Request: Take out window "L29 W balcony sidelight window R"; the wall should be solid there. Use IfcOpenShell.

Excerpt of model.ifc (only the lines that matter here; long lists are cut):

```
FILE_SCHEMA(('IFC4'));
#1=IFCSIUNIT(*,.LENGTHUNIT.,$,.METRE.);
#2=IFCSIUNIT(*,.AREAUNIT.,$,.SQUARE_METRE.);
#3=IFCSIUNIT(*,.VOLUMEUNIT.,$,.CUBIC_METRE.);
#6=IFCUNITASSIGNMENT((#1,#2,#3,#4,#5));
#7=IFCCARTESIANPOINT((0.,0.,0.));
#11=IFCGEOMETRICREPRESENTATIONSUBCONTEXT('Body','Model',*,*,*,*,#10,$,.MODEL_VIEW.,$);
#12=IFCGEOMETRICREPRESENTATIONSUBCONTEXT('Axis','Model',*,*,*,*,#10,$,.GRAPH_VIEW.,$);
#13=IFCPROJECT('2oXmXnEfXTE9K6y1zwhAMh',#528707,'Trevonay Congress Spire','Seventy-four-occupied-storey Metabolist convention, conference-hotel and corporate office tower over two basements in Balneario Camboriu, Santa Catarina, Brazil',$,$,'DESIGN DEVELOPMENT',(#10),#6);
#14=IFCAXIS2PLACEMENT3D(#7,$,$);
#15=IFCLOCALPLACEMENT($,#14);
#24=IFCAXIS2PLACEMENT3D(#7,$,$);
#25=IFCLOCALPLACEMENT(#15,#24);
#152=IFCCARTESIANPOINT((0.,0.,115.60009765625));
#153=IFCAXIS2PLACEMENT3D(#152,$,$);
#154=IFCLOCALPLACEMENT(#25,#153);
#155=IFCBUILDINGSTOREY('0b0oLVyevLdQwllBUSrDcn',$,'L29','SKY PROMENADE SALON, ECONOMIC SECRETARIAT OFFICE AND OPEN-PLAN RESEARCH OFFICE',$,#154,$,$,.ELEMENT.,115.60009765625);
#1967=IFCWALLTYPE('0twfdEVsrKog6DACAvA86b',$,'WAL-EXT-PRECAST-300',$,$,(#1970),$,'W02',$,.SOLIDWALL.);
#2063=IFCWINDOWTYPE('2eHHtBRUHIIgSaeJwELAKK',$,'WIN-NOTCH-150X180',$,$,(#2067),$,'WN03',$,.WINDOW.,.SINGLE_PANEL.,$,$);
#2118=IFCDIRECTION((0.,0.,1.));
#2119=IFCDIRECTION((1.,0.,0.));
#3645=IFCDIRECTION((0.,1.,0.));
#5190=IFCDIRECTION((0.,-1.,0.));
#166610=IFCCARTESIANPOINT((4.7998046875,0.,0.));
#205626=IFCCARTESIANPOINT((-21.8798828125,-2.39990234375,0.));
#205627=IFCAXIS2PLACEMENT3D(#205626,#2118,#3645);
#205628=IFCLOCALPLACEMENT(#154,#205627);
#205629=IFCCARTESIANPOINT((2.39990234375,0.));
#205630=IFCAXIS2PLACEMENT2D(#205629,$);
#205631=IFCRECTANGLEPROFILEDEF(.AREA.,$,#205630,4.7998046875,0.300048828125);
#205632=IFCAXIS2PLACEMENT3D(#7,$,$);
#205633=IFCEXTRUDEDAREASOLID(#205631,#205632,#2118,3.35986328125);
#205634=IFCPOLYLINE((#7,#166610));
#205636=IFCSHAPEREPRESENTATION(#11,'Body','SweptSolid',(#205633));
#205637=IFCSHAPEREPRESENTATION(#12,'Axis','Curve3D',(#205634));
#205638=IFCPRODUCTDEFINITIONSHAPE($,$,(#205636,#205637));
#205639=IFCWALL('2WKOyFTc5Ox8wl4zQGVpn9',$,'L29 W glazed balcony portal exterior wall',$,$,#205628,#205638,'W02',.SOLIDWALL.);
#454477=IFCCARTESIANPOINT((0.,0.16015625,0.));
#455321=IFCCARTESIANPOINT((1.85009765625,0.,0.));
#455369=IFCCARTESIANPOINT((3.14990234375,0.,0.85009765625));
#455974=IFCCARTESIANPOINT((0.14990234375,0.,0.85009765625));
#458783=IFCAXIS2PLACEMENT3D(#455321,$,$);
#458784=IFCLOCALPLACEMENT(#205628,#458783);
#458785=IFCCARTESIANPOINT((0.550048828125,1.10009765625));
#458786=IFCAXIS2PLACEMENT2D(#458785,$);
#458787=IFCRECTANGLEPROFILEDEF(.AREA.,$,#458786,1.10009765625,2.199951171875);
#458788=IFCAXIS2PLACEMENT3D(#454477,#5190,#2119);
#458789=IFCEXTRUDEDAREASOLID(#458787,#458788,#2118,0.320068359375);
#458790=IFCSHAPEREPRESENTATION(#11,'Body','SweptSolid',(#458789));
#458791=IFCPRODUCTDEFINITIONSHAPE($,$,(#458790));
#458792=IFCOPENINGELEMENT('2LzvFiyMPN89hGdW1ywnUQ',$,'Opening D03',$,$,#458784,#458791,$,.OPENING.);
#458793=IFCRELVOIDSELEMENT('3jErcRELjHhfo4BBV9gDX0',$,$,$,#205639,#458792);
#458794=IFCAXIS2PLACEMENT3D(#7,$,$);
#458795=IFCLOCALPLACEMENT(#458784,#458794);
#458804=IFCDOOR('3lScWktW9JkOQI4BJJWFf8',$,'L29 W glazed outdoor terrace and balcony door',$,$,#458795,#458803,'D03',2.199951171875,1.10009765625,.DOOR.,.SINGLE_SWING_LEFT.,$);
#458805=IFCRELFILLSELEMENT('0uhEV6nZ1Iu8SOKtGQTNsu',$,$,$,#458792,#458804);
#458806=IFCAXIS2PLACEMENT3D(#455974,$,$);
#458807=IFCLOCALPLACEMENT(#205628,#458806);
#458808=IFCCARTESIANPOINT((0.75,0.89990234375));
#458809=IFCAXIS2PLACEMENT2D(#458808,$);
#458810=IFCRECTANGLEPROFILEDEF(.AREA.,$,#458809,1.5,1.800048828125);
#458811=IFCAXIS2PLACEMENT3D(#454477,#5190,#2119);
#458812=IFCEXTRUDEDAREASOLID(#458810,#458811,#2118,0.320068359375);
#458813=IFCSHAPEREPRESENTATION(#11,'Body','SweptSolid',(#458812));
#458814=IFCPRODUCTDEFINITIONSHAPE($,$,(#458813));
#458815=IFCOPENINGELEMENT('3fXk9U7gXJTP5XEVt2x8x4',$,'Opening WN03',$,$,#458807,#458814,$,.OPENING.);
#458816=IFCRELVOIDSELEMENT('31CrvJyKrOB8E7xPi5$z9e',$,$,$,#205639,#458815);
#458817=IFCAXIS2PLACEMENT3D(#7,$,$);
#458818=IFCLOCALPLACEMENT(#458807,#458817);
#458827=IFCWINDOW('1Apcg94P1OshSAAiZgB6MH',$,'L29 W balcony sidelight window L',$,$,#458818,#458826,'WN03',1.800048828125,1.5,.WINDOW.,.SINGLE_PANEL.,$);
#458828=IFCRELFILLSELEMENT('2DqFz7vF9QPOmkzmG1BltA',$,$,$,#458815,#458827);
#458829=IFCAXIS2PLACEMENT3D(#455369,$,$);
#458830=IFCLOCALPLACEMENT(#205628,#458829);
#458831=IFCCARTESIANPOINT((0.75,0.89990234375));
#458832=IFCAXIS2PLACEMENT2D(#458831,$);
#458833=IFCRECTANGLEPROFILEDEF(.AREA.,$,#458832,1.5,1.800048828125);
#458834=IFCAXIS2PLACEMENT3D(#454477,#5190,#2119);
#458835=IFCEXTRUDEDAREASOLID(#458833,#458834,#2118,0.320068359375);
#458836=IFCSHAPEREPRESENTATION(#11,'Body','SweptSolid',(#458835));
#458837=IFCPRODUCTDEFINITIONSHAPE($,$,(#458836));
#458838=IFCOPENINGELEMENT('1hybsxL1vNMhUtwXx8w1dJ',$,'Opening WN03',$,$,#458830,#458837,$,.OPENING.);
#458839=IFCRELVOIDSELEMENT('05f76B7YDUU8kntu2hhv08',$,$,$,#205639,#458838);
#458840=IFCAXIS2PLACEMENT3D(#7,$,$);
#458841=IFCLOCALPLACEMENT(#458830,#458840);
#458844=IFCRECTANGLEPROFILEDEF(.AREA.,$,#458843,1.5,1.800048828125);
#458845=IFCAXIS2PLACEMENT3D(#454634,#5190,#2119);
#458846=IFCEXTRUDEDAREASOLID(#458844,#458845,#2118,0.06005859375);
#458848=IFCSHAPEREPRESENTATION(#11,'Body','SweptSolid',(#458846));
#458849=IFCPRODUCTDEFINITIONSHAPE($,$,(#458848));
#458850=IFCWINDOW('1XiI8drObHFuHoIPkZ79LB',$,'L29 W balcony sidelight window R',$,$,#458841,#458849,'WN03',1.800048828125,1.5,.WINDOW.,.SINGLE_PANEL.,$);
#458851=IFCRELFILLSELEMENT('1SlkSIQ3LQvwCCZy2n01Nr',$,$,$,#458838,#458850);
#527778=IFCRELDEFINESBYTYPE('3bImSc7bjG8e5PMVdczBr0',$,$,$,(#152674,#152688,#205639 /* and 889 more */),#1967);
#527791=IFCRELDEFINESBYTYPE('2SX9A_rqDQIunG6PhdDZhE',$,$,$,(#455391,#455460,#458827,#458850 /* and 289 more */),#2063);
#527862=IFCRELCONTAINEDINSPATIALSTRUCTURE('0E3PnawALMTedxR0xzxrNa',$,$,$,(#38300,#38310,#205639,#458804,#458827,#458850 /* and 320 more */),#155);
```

```python
import ifcopenshell
import ifcopenshell.api.feature
import ifcopenshell.api.root
import ifcopenshell.geom
import ifcopenshell.util.shape

model = ifcopenshell.open("model.ifc")
settings = ifcopenshell.geom.settings()


def volume(element):
    """Net volume in cubic metres, openings subtracted."""
    shape = ifcopenshell.geom.create_shape(settings, element)
    return ifcopenshell.util.shape.get_volume(shape.geometry)


window = model.by_guid("1XiI8drObHFuHoIPkZ79LB")
opening = window.FillsVoids[0].RelatingOpeningElement
wall = opening.VoidsElements[0].RelatingBuildingElement
before = volume(wall)

ifcopenshell.api.root.remove_product(model, product=window)
ifcopenshell.api.feature.remove_feature(model, feature=opening)

after = volume(wall)

print(f"wall volume {before:.3f} -> {after:.3f} m3")

model.write("model-out.ifc")
```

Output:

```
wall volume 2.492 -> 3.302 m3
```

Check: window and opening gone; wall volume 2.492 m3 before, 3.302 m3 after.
